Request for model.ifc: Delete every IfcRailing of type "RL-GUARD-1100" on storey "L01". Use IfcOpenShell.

First a look at what the model holds.

```python
import ifcopenshell
import ifcopenshell.util.element

model = ifcopenshell.open("model.ifc")
print(model.schema)
storey = next(s for s in model.by_type("IfcBuildingStorey") if s.Name == "L01")
railings = [e for e in ifcopenshell.util.element.get_decomposition(storey) if e.is_a("IfcRailing")]
seen = {}
for e in railings:
    element_type = ifcopenshell.util.element.get_type(e)
    name = element_type.Name if element_type not in (None, e) else None
    seen[name] = seen.get(name, 0) + 1
for name, count in sorted(seen.items(), key=str):
    print(count, "x", name)
```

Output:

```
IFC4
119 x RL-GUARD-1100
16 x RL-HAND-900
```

```python
import ifcopenshell
import ifcopenshell.api.root
import ifcopenshell.util.element

model = ifcopenshell.open("model.ifc")

storey = next(s for s in model.by_type("IfcBuildingStorey") if s.Name == "L01")
railings = [e for e in ifcopenshell.util.element.get_decomposition(storey) if e.is_a("IfcRailing")]
targets = [e for e in railings if (t := ifcopenshell.util.element.get_type(e)) not in (None, e) and t.Name == "RL-GUARD-1100"]

for e in targets:
    ifcopenshell.api.root.remove_product(model, product=e)
print(len(targets), "removed")

model.write("model-out.ifc")
```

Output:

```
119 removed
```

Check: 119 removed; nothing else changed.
